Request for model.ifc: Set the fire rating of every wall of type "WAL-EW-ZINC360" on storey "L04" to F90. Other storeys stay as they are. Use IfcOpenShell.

First a look at what the model holds.

```python
import ifcopenshell
import ifcopenshell.util.element

model = ifcopenshell.open("model.ifc")
print(model.schema)
storey = next(s for s in model.by_type("IfcBuildingStorey") if s.Name == "L04")
walls = [e for e in ifcopenshell.util.element.get_decomposition(storey) if e.is_a("IfcWall")]
seen = {}
for e in walls:
    element_type = ifcopenshell.util.element.get_type(e)
    key = (element_type.Name if element_type != e and element_type else None, ifcopenshell.util.element.get_pset(e, "Pset_WallCommon", "FireRating"))
    seen[key] = seen.get(key, 0) + 1
for (name, value), count in sorted(seen.items(), key=str):
    print(count, "x", name, "|", value)
```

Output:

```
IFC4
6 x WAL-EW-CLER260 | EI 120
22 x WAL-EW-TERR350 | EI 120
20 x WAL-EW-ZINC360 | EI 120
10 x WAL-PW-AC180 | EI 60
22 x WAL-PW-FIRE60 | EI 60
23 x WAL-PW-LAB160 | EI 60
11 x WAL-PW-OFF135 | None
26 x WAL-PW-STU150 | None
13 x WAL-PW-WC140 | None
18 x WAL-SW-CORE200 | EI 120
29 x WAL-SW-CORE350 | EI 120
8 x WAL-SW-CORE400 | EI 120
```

```python
import ifcopenshell
import ifcopenshell.api.pset
import ifcopenshell.util.element

model = ifcopenshell.open("model.ifc")

storey = next(s for s in model.by_type("IfcBuildingStorey") if s.Name == "L04")
walls = [e for e in ifcopenshell.util.element.get_decomposition(storey) if e.is_a("IfcWall")]

count = 0
for e in walls:
    element_type = ifcopenshell.util.element.get_type(e)
    if element_type in (None, e) or element_type.Name != "WAL-EW-ZINC360":
        continue
    # add_pset returns the element's existing set when there is one.
    pset = ifcopenshell.api.pset.add_pset(model, product=e, name="Pset_WallCommon")
    ifcopenshell.api.pset.edit_pset(model, pset=pset, properties={"FireRating": "F90"})
    count += 1

print(count, "walls updated")

model.write("model_edited.ifc")
```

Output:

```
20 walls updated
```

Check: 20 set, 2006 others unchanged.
